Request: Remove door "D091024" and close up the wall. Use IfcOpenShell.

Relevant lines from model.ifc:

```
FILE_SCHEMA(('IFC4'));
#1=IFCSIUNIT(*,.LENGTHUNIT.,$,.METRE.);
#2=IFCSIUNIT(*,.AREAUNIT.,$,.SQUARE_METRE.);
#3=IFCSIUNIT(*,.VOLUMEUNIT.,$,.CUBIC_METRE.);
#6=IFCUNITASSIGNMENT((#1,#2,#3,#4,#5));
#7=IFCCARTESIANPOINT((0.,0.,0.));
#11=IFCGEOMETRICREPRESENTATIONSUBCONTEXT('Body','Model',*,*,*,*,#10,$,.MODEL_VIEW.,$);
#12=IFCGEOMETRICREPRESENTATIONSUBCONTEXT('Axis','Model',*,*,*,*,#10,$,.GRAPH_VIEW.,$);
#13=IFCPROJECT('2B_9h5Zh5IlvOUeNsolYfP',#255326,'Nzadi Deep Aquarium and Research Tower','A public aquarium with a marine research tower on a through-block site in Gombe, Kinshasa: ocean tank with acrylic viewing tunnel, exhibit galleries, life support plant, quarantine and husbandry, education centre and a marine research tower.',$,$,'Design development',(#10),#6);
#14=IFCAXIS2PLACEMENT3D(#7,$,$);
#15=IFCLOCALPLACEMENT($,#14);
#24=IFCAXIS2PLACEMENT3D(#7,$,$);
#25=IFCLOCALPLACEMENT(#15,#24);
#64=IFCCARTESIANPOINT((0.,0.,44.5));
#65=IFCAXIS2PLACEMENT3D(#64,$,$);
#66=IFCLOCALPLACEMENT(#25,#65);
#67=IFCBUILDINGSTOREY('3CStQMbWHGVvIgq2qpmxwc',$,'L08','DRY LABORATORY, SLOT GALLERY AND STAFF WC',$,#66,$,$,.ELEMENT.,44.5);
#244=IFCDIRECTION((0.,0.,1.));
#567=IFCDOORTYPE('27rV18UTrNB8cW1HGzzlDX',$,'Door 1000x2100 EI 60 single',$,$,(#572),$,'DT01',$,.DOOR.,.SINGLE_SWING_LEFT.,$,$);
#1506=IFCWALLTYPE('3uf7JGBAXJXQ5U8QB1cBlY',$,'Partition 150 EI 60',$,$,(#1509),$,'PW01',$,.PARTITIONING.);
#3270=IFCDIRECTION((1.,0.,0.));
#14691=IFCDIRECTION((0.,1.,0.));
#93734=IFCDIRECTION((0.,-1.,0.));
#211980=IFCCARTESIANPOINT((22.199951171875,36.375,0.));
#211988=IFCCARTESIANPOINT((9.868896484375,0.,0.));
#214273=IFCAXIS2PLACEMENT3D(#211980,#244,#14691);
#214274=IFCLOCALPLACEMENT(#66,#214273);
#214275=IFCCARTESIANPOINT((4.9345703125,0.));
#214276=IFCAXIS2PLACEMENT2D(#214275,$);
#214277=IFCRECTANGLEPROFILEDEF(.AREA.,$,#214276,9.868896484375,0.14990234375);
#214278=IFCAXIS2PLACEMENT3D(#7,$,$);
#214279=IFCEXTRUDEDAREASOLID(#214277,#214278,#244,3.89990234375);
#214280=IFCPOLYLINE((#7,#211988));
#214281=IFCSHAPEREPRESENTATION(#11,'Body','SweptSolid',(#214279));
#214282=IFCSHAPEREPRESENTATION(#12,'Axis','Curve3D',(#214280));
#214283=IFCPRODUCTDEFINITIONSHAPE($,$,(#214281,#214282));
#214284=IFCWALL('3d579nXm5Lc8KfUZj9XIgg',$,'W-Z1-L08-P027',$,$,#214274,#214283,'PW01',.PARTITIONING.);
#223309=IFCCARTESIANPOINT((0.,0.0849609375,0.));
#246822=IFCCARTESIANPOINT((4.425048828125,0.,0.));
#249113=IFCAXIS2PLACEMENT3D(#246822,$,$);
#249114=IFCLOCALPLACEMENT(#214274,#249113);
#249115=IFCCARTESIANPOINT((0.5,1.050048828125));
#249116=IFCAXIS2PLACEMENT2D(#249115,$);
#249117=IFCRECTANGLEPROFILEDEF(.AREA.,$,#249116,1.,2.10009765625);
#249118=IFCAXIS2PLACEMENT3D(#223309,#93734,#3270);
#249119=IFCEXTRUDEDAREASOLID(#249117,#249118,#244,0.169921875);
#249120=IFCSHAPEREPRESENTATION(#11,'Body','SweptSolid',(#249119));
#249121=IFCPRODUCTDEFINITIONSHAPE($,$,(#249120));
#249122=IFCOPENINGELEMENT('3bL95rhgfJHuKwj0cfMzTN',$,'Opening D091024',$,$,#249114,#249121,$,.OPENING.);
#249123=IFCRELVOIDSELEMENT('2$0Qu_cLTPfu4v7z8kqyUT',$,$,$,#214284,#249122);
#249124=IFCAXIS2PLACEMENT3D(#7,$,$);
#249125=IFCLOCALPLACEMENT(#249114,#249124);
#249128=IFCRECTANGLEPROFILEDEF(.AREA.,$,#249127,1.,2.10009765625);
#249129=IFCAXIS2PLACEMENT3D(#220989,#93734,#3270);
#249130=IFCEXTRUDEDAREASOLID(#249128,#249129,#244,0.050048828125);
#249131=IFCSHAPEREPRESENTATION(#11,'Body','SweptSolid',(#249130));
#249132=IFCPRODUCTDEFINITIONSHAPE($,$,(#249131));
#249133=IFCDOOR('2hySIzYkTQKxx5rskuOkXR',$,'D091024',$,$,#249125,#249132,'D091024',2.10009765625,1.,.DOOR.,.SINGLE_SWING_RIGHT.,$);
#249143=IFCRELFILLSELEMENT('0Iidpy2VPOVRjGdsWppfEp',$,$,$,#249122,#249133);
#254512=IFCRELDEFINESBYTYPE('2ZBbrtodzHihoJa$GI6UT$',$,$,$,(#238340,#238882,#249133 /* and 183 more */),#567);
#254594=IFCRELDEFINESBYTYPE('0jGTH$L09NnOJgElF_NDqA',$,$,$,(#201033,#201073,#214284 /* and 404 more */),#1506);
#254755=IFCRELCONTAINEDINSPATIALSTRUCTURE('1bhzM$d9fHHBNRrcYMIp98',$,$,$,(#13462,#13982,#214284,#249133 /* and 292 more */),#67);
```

```python
import ifcopenshell
import ifcopenshell.api.feature
import ifcopenshell.api.root
import ifcopenshell.geom
import ifcopenshell.util.shape

model = ifcopenshell.open("model.ifc")
settings = ifcopenshell.geom.settings()


def volume(element):
    """Net volume in cubic metres, openings subtracted."""
    shape = ifcopenshell.geom.create_shape(settings, element)
    return ifcopenshell.util.shape.get_volume(shape.geometry)


door = model.by_id(249133)
opening = door.FillsVoids[0].RelatingOpeningElement
wall = opening.VoidsElements[0].RelatingBuildingElement
before = volume(wall)

ifcopenshell.api.root.remove_product(model, product=door)
ifcopenshell.api.feature.remove_feature(model, feature=opening)

after = volume(wall)

print(f"wall volume {before:.3f} -> {after:.3f} m3")

model.write("model-out.ifc")
```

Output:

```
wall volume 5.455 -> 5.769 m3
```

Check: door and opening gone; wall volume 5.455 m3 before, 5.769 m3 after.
